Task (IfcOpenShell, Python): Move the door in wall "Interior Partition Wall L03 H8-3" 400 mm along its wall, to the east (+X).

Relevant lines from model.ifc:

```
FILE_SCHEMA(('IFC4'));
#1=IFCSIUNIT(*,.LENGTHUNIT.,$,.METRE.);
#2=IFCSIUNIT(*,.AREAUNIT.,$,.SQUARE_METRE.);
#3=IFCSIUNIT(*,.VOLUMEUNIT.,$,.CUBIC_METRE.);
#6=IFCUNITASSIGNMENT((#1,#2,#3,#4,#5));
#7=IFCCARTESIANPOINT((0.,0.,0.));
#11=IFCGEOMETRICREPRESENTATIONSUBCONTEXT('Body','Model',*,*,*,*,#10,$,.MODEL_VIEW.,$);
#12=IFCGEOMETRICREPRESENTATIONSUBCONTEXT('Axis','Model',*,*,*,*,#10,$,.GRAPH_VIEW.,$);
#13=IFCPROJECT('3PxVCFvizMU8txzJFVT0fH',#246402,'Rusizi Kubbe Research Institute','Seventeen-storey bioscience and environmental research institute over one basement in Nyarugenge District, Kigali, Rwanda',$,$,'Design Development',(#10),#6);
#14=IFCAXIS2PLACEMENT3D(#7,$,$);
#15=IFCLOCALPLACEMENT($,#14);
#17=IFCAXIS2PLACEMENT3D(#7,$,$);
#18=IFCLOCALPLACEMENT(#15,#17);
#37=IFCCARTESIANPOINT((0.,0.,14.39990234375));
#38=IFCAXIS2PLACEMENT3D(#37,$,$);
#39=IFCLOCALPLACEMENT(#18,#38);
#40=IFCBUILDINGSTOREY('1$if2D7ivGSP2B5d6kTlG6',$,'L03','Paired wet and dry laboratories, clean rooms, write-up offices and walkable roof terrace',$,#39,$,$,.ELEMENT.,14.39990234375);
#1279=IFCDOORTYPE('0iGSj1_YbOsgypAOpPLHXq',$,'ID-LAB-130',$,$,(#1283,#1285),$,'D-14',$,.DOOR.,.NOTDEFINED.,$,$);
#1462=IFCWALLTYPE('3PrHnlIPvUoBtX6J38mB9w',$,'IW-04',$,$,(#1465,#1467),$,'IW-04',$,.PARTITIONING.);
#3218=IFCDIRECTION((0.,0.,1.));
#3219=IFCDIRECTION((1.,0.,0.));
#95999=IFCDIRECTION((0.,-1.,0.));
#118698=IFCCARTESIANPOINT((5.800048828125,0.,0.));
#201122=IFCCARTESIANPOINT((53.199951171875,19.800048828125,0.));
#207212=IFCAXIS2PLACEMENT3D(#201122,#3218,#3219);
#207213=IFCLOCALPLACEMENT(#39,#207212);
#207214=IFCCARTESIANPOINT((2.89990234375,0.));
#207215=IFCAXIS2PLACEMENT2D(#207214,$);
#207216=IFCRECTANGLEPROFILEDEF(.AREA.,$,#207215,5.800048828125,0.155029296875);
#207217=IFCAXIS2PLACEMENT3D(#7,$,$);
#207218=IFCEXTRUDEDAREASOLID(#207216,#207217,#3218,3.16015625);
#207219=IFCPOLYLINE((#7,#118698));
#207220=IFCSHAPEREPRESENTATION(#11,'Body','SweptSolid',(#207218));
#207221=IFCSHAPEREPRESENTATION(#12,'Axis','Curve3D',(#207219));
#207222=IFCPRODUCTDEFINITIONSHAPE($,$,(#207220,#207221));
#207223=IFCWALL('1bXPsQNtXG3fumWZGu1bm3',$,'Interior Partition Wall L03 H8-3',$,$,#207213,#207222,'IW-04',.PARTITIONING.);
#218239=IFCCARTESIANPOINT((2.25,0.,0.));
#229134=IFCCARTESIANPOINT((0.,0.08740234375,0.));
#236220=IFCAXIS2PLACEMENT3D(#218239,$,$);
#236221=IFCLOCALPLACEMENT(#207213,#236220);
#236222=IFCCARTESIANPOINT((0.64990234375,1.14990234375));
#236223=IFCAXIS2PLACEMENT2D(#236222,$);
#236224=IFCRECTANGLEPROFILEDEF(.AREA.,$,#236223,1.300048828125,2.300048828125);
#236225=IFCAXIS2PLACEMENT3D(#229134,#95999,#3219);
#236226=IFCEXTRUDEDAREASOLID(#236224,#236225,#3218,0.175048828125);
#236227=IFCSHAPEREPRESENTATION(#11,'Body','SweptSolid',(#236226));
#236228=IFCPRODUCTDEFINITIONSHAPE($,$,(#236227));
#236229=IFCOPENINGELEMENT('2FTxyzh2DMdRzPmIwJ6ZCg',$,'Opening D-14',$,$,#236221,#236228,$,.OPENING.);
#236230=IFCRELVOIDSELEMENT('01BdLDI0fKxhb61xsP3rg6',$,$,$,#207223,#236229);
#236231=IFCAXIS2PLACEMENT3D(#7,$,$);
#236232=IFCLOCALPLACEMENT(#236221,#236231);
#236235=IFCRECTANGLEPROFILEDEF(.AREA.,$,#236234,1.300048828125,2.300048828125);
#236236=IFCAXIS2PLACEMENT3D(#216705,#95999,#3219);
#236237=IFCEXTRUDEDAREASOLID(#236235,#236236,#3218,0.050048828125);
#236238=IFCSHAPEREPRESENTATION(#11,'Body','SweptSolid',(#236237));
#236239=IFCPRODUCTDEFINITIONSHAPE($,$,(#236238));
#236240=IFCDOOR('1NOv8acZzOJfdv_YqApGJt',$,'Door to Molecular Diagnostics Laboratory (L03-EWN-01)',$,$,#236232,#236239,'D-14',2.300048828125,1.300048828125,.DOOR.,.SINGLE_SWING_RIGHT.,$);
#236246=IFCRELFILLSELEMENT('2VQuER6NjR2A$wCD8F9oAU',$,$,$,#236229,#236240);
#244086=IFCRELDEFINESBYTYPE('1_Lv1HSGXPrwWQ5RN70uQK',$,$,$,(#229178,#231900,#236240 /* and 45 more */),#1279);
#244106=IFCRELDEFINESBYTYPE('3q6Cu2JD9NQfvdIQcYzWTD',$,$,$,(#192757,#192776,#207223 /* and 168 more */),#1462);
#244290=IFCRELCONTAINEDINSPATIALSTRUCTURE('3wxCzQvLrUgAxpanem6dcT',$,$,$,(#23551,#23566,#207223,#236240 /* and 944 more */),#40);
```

```python
import ifcopenshell
import ifcopenshell.api.geometry
import ifcopenshell.util.placement
import ifcopenshell.util.unit

model = ifcopenshell.open("model.ifc")
unit_scale = ifcopenshell.util.unit.calculate_unit_scale(model)

door = model.by_id(236240)
opening = door.FillsVoids[0].RelatingOpeningElement
wall = opening.VoidsElements[0].RelatingBuildingElement

wall_matrix = ifcopenshell.util.placement.get_local_placement(wall.ObjectPlacement)
shift = wall_matrix[:3, 0] * 0.4 / unit_scale
before = ifcopenshell.util.placement.get_local_placement(door.ObjectPlacement)[:3, 3].copy()

# The door is placed relative to its opening, so it follows when the opening moves.
matrix = ifcopenshell.util.placement.get_local_placement(opening.ObjectPlacement)
matrix[:3, 3] += shift
ifcopenshell.api.geometry.edit_object_placement(
    model, product=opening, matrix=matrix, is_si=False, should_transform_children=True
)

after = ifcopenshell.util.placement.get_local_placement(door.ObjectPlacement)[:3, 3]
print("door moved by", (after - before).round(3) + 0.0)

model.write("model_updated.ifc")
```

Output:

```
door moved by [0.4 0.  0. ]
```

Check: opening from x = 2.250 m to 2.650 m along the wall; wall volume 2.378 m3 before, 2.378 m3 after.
